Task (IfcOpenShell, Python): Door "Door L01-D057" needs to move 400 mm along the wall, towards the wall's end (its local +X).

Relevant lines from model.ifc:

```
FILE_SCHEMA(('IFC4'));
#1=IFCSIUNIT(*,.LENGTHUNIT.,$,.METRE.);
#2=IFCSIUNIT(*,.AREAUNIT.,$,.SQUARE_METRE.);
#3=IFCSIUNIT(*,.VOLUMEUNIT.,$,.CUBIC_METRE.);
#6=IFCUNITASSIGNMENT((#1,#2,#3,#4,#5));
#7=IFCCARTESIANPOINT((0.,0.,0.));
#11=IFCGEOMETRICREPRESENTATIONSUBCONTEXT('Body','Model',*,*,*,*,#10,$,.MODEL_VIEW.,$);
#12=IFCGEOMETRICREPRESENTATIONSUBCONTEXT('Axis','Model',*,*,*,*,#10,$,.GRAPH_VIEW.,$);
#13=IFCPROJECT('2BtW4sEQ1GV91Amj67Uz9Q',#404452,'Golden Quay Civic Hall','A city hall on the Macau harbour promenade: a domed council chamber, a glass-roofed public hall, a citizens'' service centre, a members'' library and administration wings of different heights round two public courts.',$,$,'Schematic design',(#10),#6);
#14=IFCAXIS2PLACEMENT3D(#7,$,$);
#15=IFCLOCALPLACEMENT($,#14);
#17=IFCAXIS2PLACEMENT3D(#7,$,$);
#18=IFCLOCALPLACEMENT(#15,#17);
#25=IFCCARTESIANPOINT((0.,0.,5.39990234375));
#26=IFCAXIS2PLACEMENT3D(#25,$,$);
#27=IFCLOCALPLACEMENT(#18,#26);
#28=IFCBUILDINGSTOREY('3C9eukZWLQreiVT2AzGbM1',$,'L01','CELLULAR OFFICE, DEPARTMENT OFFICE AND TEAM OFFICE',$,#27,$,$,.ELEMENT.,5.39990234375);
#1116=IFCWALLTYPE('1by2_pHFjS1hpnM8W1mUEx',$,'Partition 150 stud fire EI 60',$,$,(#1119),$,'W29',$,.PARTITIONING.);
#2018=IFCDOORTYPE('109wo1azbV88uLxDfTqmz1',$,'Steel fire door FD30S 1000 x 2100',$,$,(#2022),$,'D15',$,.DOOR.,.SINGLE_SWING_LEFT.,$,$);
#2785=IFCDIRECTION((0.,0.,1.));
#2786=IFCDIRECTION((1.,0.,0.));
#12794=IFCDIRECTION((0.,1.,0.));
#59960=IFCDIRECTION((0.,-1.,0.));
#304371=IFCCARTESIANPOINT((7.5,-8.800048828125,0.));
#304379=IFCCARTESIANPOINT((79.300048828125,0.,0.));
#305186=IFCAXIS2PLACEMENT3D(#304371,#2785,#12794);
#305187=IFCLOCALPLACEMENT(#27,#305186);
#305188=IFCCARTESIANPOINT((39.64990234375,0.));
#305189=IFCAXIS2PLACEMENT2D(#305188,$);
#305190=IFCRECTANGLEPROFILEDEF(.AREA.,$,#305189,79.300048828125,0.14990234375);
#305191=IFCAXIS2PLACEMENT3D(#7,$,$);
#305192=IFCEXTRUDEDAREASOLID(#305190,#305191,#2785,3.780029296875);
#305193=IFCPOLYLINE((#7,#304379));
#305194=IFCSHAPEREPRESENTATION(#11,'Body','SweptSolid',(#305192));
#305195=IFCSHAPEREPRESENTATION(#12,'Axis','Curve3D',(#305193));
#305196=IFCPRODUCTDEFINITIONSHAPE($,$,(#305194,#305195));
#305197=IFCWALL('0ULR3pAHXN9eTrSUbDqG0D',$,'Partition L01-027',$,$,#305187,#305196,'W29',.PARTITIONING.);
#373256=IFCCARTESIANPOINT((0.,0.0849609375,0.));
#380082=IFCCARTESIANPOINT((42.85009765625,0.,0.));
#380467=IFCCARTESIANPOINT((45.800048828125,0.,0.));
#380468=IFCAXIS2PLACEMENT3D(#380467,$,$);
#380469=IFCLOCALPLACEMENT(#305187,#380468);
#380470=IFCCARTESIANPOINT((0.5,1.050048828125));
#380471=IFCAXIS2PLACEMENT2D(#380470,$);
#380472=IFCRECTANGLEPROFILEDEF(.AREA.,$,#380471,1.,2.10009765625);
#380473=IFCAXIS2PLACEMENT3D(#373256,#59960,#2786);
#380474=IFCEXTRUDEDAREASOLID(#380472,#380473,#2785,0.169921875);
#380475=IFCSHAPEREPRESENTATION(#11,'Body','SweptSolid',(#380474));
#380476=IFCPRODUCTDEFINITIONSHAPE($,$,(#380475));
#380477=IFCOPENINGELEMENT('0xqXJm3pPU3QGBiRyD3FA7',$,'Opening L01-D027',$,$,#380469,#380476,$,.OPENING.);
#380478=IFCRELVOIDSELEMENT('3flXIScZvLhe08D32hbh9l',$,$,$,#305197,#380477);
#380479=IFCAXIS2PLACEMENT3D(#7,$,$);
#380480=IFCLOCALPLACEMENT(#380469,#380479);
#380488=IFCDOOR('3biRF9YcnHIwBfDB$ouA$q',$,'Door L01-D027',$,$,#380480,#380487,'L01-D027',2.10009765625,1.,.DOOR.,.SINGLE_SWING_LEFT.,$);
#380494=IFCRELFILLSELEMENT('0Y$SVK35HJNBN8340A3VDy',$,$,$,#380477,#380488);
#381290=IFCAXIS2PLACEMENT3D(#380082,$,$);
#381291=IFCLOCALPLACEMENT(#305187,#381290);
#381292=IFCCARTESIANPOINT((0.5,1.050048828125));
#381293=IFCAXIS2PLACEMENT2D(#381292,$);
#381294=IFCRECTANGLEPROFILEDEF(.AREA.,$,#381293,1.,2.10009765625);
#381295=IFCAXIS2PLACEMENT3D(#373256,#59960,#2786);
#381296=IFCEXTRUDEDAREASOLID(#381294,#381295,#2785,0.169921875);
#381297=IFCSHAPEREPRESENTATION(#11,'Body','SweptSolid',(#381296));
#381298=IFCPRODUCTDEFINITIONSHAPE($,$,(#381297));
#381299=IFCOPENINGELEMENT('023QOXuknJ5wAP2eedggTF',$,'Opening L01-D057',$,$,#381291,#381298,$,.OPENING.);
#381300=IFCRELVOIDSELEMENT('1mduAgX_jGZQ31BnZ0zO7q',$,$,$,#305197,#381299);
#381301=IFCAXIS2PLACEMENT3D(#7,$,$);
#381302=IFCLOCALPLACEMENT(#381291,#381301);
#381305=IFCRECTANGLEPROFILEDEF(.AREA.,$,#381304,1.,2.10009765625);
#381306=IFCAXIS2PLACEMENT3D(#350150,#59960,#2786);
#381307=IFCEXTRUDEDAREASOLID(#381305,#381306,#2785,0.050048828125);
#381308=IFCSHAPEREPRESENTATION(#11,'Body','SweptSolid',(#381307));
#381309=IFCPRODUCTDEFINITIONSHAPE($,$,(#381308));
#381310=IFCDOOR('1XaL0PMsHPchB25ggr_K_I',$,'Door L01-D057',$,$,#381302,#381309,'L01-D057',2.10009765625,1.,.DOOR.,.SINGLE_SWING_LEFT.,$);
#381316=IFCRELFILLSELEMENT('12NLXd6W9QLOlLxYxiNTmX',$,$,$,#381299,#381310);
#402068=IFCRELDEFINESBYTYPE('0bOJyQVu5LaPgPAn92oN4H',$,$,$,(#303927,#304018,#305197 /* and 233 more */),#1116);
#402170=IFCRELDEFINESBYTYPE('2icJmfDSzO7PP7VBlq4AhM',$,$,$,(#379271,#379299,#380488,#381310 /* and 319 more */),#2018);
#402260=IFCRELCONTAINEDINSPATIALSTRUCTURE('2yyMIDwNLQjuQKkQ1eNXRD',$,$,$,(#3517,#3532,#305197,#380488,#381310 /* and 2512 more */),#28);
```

```python
import ifcopenshell
import ifcopenshell.api.geometry
import ifcopenshell.util.placement
import ifcopenshell.util.unit

model = ifcopenshell.open("model.ifc")
unit_scale = ifcopenshell.util.unit.calculate_unit_scale(model)

door = model.by_guid("1XaL0PMsHPchB25ggr_K_I")
opening = door.FillsVoids[0].RelatingOpeningElement
wall = opening.VoidsElements[0].RelatingBuildingElement

wall_matrix = ifcopenshell.util.placement.get_local_placement(wall.ObjectPlacement)
shift = wall_matrix[:3, 0] * 0.4 / unit_scale
before = ifcopenshell.util.placement.get_local_placement(door.ObjectPlacement)[:3, 3].copy()

# The door is placed relative to its opening, so it follows when the opening moves.
matrix = ifcopenshell.util.placement.get_local_placement(opening.ObjectPlacement)
matrix[:3, 3] += shift
ifcopenshell.api.geometry.edit_object_placement(
    model, product=opening, matrix=matrix, is_si=False, should_transform_children=True
)

after = ifcopenshell.util.placement.get_local_placement(door.ObjectPlacement)[:3, 3]
print("door moved by", (after - before).round(3) + 0.0)

model.write("model_updated.ifc")
```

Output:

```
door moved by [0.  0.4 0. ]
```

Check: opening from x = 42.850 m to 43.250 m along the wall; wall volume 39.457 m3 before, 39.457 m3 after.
